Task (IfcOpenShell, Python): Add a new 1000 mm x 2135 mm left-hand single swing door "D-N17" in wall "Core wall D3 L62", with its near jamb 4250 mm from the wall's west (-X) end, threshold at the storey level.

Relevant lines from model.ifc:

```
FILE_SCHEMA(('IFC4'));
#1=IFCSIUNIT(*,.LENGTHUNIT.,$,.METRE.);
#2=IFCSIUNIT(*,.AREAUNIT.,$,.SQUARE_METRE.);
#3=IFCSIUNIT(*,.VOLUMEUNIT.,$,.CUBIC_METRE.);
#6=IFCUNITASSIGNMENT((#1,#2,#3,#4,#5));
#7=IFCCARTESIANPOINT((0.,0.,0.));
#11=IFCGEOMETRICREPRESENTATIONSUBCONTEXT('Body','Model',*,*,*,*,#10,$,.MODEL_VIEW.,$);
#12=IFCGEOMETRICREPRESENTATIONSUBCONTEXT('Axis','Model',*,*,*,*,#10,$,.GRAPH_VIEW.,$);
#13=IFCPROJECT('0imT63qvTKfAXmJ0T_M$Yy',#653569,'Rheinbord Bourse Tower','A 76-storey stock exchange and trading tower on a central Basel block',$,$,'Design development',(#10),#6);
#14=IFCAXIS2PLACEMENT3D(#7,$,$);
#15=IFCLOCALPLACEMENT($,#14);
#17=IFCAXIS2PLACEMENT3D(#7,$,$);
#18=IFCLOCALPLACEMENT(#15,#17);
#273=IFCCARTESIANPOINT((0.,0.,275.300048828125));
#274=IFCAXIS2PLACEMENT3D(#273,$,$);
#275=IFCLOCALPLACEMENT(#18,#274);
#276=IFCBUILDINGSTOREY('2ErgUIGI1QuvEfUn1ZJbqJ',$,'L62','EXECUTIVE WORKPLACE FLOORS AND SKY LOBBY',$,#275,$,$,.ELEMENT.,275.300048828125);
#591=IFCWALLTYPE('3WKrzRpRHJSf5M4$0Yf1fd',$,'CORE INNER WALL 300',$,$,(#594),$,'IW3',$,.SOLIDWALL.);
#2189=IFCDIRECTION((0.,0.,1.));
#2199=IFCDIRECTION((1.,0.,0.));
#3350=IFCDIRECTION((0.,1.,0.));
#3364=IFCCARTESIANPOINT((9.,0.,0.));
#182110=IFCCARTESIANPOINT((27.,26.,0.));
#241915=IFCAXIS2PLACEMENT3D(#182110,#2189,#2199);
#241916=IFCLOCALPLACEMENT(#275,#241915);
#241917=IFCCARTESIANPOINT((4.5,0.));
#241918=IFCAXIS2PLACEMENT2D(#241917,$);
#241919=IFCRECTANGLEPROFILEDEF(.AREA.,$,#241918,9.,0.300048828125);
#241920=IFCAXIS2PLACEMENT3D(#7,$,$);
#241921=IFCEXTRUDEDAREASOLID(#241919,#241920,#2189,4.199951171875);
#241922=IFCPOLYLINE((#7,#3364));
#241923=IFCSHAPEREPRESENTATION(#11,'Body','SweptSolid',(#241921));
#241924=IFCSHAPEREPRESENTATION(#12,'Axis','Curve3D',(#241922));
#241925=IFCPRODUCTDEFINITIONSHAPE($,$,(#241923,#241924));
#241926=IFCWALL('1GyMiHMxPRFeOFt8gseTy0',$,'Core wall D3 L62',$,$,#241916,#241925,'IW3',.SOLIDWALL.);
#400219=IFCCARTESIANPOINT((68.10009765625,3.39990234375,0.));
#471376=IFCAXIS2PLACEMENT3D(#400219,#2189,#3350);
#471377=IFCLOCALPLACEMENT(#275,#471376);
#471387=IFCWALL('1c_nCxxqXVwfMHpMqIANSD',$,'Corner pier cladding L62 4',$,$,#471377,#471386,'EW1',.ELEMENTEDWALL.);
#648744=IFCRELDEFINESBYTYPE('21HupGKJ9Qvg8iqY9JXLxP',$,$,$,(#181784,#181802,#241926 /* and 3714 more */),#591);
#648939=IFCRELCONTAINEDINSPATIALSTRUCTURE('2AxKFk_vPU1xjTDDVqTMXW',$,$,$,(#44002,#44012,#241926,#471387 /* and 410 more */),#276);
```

```python
import numpy as np
import ifcopenshell
import ifcopenshell.api.feature
import ifcopenshell.api.geometry
import ifcopenshell.api.root
import ifcopenshell.api.spatial
import ifcopenshell.geom
import ifcopenshell.util.element
import ifcopenshell.util.placement
import ifcopenshell.util.representation
import ifcopenshell.util.shape
import ifcopenshell.util.unit

model = ifcopenshell.open("model.ifc")
unit_scale = ifcopenshell.util.unit.calculate_unit_scale(model)
settings = ifcopenshell.geom.settings()


def volume(element):
    """Net volume in cubic metres, openings subtracted."""
    shape = ifcopenshell.geom.create_shape(settings, element)
    return ifcopenshell.util.shape.get_volume(shape.geometry)


wall = model.by_guid("1GyMiHMxPRFeOFt8gseTy0")
storey = ifcopenshell.util.element.get_container(wall, ifc_class="IfcBuildingStorey")
context = ifcopenshell.util.representation.get_context(model, "Model", "Body", "MODEL_VIEW")
before = volume(wall)

width, height, from_end, sill = 1, 2.135, 4.25, 0.0  # metres

# The wall runs along its own X axis, and the end named is its -X end.
wall_shape = ifcopenshell.geom.create_shape(settings, wall)
x, y, z = ifcopenshell.util.shape.get_vertices(wall_shape.geometry).T
start = x.min() + from_end
face, thickness = float(y.min()), float(y.max() - y.min())
wall_matrix = ifcopenshell.util.placement.get_local_placement(wall.ObjectPlacement)
level = ifcopenshell.util.placement.get_local_placement(storey.ObjectPlacement)[2, 3]


def in_wall(x, y):
    """Placement at x, y metres in the wall's axes, at sill height."""
    matrix = wall_matrix.copy()
    matrix[:, 3] = wall_matrix @ np.array([x / unit_scale, y / unit_scale, 0.0, 1.0])
    matrix[2, 3] = level + sill / unit_scale
    return matrix


# Opening: a box that overshoots both wall faces by 50 mm.
opening = ifcopenshell.api.root.create_entity(model, ifc_class="IfcOpeningElement", predefined_type="OPENING")
box = ifcopenshell.api.geometry.add_wall_representation(
    model, context=context, length=width, height=height, thickness=thickness + 0.1
)
ifcopenshell.api.geometry.assign_representation(model, product=opening, representation=box)
ifcopenshell.api.geometry.edit_object_placement(model, product=opening, matrix=in_wall(start, face - 0.05), is_si=False)
ifcopenshell.api.feature.add_feature(model, feature=opening, element=wall)

door = ifcopenshell.api.root.create_entity(model, ifc_class="IfcDoor", name="D-N17", predefined_type="DOOR")
door.OverallWidth, door.OverallHeight = width / unit_scale, height / unit_scale
door.OperationType = "SINGLE_SWING_LEFT"
body = ifcopenshell.api.geometry.add_door_representation(
    model,
    context=context,
    overall_width=door.OverallWidth,
    overall_height=door.OverallHeight,
    operation_type="SINGLE_SWING_LEFT",
    lining_properties={"LiningDepth": thickness / unit_scale, "ThresholdDepth": thickness / unit_scale},
)
ifcopenshell.api.geometry.assign_representation(model, product=door, representation=body)
ifcopenshell.api.spatial.assign_container(model, products=[door], relating_structure=storey)
ifcopenshell.api.feature.add_filling(model, opening=opening, element=door)

# The lining spans the wall, so the door starts at the wall face.
ifcopenshell.api.geometry.edit_object_placement(model, product=door, matrix=in_wall(start, face), is_si=False)

after = volume(wall)

print(f"wall volume {before:.3f} -> {after:.3f} m3")

model.write("model_rev.ifc")
```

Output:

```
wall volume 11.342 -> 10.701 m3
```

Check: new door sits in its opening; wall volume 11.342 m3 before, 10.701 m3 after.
